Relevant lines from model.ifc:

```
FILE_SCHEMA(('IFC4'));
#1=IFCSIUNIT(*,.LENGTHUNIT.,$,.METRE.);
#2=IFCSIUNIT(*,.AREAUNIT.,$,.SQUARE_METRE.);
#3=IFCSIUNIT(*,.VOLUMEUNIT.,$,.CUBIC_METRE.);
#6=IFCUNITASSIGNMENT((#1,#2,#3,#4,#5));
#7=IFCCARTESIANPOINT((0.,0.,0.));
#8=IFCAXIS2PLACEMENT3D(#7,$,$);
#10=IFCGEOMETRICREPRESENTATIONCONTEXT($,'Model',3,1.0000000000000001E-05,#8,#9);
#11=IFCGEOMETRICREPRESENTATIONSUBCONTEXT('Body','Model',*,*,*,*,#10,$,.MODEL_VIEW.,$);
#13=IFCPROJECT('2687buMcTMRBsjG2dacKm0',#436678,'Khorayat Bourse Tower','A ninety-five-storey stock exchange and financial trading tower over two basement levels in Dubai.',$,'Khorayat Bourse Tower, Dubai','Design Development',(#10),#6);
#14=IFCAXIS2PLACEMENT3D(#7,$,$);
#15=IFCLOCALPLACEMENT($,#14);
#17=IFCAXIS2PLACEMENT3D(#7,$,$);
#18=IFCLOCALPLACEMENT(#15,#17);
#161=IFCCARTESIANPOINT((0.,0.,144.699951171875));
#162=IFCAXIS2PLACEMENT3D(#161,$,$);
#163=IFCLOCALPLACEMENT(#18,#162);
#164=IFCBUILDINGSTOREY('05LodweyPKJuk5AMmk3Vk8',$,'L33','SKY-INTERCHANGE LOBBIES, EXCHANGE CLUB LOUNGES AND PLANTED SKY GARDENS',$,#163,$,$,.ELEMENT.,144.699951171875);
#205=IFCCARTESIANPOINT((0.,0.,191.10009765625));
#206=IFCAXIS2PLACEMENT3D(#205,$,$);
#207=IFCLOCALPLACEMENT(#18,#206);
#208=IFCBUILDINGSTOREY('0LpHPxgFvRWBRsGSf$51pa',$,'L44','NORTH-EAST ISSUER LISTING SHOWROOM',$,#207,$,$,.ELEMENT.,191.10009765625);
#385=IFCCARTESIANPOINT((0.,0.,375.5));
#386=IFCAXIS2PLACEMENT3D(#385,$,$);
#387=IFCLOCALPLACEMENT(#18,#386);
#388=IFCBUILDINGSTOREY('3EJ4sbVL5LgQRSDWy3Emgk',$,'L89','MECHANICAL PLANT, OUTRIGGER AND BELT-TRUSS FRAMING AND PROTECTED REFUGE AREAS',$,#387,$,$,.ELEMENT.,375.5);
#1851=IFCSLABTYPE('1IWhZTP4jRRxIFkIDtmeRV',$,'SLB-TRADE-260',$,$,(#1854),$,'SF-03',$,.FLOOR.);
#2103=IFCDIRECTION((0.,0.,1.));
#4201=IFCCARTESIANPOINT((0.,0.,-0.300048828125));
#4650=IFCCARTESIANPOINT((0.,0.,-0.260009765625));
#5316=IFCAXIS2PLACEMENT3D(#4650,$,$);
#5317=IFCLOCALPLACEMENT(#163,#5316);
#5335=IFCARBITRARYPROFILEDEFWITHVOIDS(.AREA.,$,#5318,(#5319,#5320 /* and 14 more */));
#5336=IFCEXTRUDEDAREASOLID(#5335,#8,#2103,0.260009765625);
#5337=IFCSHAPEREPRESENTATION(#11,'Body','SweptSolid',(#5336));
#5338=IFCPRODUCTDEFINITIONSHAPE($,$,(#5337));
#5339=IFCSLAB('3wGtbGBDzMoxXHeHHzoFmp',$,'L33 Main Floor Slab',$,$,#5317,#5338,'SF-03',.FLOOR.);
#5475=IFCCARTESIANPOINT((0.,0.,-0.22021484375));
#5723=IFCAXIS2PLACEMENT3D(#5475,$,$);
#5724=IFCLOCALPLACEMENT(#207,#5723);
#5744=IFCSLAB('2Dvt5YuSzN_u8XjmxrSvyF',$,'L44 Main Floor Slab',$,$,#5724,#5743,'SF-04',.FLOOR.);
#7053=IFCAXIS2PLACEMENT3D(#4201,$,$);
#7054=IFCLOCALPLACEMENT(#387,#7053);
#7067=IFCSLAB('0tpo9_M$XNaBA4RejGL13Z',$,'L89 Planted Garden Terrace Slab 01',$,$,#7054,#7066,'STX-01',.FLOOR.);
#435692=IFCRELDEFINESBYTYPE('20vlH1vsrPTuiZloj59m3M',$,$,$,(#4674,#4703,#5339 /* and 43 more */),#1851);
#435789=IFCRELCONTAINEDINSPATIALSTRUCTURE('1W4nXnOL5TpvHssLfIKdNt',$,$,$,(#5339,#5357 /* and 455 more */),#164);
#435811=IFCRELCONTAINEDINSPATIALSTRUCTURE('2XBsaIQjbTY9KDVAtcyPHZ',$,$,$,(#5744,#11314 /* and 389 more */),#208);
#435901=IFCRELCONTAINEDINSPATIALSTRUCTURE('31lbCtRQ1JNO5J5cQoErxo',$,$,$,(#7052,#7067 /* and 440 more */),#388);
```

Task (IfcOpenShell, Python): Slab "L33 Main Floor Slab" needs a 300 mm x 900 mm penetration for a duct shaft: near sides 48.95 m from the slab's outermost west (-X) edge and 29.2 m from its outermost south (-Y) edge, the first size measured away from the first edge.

```python
import numpy as np
import ifcopenshell
import ifcopenshell.api.feature
import ifcopenshell.api.geometry
import ifcopenshell.api.root
import ifcopenshell.geom
import ifcopenshell.util.placement
import ifcopenshell.util.representation
import ifcopenshell.util.shape
import ifcopenshell.util.unit

model = ifcopenshell.open("model.ifc")
unit_scale = ifcopenshell.util.unit.calculate_unit_scale(model)
settings = ifcopenshell.geom.settings()


def volume(element):
    """Net volume in cubic metres, openings subtracted."""
    shape = ifcopenshell.geom.create_shape(settings, element)
    return ifcopenshell.util.shape.get_volume(shape.geometry)


slab = model.by_guid("3wGtbGBDzMoxXHeHHzoFmp")
before = volume(slab)

# Extent in the slab's own axes, in metres. The edges named are its -X and -Y sides.
slab_shape = ifcopenshell.geom.create_shape(settings, slab)
vertices = ifcopenshell.util.shape.get_vertices(slab_shape.geometry)
x_min, y_min, bottom = vertices.min(axis=0)
top = vertices[:, 2].max()

opening = ifcopenshell.api.root.create_entity(model, ifc_class="IfcOpeningElement", name="Duct shaft opening", predefined_type="OPENING")
context = ifcopenshell.util.representation.get_context(model, "Model", "Body", "MODEL_VIEW")
width, depth = 0.3, 0.9
outline = [(0.0, 0.0), (width, 0.0), (width, depth), (0.0, depth), (0.0, 0.0)]
# Overshoot both faces by 50 mm so the cut is clean.
shape = ifcopenshell.api.geometry.add_slab_representation(
    model, context=context, depth=top - bottom + 0.1, polyline=outline
)
ifcopenshell.api.geometry.assign_representation(model, product=opening, representation=shape)

matrix = ifcopenshell.util.placement.get_local_placement(slab.ObjectPlacement)
matrix[:, 3] = matrix @ np.append(np.array([x_min + 48.95, y_min + 29.2, bottom - 0.05]) / unit_scale, 1.0)
ifcopenshell.api.geometry.edit_object_placement(model, product=opening, matrix=matrix, is_si=False)
ifcopenshell.api.feature.add_feature(model, feature=opening, element=slab)

after = volume(slab)

print(f"slab volume {before:.3f} -> {after:.3f} m3")

model.write("model-out.ifc")
```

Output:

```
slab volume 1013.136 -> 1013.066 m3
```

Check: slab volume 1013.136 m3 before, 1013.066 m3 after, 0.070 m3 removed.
